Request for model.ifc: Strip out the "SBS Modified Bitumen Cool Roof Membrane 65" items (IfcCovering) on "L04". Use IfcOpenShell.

First a look at what the model holds.

```python
import ifcopenshell
import ifcopenshell.util.element

model = ifcopenshell.open("model.ifc")
print(model.schema)
storey = next(s for s in model.by_type("IfcBuildingStorey") if s.Name == "L04")
coverings = [e for e in ifcopenshell.util.element.get_decomposition(storey) if e.is_a("IfcCovering")]
seen = {}
for e in coverings:
    element_type = ifcopenshell.util.element.get_type(e)
    name = element_type.Name if element_type not in (None, e) else None
    seen[name] = seen.get(name, 0) + 1
for name, count in sorted(seen.items(), key=str):
    print(count, "x", name)
```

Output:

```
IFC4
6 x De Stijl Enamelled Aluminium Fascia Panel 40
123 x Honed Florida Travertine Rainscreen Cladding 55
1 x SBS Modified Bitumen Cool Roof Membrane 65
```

```python
import ifcopenshell
import ifcopenshell.api.root
import ifcopenshell.util.element

model = ifcopenshell.open("model.ifc")

storey = next(s for s in model.by_type("IfcBuildingStorey") if s.Name == "L04")
coverings = [e for e in ifcopenshell.util.element.get_decomposition(storey) if e.is_a("IfcCovering")]
targets = [e for e in coverings if (t := ifcopenshell.util.element.get_type(e)) not in (None, e) and t.Name == "SBS Modified Bitumen Cool Roof Membrane 65"]

for e in targets:
    ifcopenshell.api.root.remove_product(model, product=e)
print(len(targets), "removed")

model.write("model_rev.ifc")
```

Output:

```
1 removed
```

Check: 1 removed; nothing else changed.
